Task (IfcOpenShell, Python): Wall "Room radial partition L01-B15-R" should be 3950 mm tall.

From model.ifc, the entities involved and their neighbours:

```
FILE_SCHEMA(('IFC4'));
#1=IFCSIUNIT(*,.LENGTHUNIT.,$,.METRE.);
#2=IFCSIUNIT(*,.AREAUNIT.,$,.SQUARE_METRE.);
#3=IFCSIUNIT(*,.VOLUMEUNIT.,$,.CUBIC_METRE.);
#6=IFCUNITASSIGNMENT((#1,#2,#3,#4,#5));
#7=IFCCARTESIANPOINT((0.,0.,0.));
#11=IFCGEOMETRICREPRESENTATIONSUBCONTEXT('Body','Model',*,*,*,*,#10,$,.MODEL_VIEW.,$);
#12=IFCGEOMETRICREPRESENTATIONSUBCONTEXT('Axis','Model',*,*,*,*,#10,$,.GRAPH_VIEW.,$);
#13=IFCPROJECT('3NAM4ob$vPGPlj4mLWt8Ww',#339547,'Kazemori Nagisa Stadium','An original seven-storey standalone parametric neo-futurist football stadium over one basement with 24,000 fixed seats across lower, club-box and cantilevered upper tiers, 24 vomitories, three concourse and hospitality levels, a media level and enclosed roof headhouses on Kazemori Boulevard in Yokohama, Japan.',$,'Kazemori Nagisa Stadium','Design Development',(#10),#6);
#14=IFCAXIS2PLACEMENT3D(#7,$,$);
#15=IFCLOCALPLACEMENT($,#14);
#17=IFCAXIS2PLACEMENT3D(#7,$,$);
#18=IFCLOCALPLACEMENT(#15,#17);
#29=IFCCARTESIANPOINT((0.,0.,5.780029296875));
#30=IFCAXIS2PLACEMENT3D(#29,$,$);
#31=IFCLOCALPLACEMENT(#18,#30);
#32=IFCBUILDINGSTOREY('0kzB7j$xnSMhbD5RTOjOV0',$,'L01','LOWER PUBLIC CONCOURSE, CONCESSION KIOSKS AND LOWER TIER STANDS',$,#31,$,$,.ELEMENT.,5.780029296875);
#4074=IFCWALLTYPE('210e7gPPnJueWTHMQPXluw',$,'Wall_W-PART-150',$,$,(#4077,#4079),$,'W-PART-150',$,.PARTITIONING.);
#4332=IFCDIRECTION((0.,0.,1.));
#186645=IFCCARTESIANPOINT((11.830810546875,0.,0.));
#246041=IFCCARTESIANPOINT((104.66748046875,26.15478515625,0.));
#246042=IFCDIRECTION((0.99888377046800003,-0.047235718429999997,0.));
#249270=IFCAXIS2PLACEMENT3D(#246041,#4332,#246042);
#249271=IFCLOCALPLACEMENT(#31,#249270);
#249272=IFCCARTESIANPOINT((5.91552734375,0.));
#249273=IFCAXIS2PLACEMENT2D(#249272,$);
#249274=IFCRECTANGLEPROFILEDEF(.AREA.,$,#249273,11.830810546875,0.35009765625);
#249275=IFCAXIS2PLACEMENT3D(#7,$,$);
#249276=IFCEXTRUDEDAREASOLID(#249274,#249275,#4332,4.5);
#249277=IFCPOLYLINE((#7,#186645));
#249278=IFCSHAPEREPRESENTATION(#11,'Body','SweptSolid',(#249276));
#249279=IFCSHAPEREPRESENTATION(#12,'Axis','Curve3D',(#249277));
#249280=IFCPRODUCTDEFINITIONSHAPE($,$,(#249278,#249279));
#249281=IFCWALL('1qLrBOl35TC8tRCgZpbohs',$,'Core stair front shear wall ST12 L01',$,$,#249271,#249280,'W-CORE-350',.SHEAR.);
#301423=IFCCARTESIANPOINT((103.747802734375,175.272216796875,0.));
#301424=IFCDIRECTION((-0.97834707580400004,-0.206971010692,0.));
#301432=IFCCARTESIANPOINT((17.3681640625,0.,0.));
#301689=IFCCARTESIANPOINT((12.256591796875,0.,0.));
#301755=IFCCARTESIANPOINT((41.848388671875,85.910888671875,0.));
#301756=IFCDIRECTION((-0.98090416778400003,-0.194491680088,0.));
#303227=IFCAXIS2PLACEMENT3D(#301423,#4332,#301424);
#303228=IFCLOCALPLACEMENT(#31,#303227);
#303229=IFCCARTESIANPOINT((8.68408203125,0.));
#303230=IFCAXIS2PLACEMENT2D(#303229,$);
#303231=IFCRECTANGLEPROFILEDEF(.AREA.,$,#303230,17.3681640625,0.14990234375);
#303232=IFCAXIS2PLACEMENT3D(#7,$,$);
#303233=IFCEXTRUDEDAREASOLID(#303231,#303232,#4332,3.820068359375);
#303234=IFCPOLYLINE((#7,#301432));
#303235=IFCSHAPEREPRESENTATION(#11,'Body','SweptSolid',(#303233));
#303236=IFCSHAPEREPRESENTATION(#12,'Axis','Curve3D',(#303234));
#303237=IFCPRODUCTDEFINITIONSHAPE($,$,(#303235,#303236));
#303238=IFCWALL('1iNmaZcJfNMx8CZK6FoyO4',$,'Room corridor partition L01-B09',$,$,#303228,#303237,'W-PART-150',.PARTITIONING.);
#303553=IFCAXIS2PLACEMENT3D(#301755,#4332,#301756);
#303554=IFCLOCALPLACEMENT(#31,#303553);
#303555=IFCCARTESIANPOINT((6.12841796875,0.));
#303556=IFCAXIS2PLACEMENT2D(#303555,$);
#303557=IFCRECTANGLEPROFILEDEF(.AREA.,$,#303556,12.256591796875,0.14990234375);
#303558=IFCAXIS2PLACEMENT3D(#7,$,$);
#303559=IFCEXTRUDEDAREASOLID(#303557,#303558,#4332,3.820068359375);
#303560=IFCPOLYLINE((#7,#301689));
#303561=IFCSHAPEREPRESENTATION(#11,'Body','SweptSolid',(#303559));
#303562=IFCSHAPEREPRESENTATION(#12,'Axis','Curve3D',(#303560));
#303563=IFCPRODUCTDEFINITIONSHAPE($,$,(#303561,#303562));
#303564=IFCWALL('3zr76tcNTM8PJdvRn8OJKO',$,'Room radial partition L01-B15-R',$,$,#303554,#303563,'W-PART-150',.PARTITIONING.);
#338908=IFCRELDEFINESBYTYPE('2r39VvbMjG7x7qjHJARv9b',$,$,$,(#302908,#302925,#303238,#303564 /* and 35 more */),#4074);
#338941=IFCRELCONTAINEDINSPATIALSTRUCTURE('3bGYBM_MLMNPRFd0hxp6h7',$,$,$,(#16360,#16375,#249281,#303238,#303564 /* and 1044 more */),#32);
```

```python
import ifcopenshell
import ifcopenshell.geom
import ifcopenshell.util.representation
import ifcopenshell.util.shape
import ifcopenshell.util.unit

model = ifcopenshell.open("model.ifc")
unit_scale = ifcopenshell.util.unit.calculate_unit_scale(model)
settings = ifcopenshell.geom.settings()


def volume(element):
    """Net volume in cubic metres, openings subtracted."""
    shape = ifcopenshell.geom.create_shape(settings, element)
    return ifcopenshell.util.shape.get_volume(shape.geometry)


wall = model.by_guid("3zr76tcNTM8PJdvRn8OJKO")
before = volume(wall)

body = ifcopenshell.util.representation.get_representation(wall, "Model", "Body")
solid = body.Items[0]
old_height = solid.Depth
solid.Depth = 3.95 / unit_scale
after = volume(wall)

print(f"height {old_height:g} -> {solid.Depth:g}, volume {before:.3f} -> {after:.3f} m3")

model.write("model-out.ifc")
```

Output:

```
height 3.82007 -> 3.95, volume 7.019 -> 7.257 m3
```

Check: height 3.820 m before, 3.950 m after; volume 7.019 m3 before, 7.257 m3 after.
